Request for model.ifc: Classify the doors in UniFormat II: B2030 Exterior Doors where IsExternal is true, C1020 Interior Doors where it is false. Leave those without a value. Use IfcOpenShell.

First a look at what the model holds.

```python
import ifcopenshell
import ifcopenshell.util.element

model = ifcopenshell.open("model.ifc")
print(model.schema)
print("classifications:", [c.Name for c in model.by_type("IfcClassification")])
values = [ifcopenshell.util.element.get_pset(e, "Pset_DoorCommon", "IsExternal") for e in model.by_type("IfcDoor")]
for value in (True, False, None):
    print("IsExternal", value, values.count(value))
```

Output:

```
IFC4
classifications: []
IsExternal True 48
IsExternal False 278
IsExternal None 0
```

```python
import ifcopenshell
import ifcopenshell.api.classification
import ifcopenshell.util.element

model = ifcopenshell.open("model.ifc")

system = ifcopenshell.api.classification.add_classification(model, classification="UniFormat II")

doors = model.by_type("IfcDoor")
external = {e: ifcopenshell.util.element.get_pset(e, "Pset_DoorCommon", "IsExternal") for e in doors}
for flag, code, name in ((True, "B2030", "Exterior Doors"), (False, "C1020", "Interior Doors")):
    products = [e for e in doors if external[e] is flag]
    ifcopenshell.api.classification.add_reference(
        model, products=products, classification=system, identification=code, name=name
    )
    print(code, len(products))

model.write("model-out.ifc")
```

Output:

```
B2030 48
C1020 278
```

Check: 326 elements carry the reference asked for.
